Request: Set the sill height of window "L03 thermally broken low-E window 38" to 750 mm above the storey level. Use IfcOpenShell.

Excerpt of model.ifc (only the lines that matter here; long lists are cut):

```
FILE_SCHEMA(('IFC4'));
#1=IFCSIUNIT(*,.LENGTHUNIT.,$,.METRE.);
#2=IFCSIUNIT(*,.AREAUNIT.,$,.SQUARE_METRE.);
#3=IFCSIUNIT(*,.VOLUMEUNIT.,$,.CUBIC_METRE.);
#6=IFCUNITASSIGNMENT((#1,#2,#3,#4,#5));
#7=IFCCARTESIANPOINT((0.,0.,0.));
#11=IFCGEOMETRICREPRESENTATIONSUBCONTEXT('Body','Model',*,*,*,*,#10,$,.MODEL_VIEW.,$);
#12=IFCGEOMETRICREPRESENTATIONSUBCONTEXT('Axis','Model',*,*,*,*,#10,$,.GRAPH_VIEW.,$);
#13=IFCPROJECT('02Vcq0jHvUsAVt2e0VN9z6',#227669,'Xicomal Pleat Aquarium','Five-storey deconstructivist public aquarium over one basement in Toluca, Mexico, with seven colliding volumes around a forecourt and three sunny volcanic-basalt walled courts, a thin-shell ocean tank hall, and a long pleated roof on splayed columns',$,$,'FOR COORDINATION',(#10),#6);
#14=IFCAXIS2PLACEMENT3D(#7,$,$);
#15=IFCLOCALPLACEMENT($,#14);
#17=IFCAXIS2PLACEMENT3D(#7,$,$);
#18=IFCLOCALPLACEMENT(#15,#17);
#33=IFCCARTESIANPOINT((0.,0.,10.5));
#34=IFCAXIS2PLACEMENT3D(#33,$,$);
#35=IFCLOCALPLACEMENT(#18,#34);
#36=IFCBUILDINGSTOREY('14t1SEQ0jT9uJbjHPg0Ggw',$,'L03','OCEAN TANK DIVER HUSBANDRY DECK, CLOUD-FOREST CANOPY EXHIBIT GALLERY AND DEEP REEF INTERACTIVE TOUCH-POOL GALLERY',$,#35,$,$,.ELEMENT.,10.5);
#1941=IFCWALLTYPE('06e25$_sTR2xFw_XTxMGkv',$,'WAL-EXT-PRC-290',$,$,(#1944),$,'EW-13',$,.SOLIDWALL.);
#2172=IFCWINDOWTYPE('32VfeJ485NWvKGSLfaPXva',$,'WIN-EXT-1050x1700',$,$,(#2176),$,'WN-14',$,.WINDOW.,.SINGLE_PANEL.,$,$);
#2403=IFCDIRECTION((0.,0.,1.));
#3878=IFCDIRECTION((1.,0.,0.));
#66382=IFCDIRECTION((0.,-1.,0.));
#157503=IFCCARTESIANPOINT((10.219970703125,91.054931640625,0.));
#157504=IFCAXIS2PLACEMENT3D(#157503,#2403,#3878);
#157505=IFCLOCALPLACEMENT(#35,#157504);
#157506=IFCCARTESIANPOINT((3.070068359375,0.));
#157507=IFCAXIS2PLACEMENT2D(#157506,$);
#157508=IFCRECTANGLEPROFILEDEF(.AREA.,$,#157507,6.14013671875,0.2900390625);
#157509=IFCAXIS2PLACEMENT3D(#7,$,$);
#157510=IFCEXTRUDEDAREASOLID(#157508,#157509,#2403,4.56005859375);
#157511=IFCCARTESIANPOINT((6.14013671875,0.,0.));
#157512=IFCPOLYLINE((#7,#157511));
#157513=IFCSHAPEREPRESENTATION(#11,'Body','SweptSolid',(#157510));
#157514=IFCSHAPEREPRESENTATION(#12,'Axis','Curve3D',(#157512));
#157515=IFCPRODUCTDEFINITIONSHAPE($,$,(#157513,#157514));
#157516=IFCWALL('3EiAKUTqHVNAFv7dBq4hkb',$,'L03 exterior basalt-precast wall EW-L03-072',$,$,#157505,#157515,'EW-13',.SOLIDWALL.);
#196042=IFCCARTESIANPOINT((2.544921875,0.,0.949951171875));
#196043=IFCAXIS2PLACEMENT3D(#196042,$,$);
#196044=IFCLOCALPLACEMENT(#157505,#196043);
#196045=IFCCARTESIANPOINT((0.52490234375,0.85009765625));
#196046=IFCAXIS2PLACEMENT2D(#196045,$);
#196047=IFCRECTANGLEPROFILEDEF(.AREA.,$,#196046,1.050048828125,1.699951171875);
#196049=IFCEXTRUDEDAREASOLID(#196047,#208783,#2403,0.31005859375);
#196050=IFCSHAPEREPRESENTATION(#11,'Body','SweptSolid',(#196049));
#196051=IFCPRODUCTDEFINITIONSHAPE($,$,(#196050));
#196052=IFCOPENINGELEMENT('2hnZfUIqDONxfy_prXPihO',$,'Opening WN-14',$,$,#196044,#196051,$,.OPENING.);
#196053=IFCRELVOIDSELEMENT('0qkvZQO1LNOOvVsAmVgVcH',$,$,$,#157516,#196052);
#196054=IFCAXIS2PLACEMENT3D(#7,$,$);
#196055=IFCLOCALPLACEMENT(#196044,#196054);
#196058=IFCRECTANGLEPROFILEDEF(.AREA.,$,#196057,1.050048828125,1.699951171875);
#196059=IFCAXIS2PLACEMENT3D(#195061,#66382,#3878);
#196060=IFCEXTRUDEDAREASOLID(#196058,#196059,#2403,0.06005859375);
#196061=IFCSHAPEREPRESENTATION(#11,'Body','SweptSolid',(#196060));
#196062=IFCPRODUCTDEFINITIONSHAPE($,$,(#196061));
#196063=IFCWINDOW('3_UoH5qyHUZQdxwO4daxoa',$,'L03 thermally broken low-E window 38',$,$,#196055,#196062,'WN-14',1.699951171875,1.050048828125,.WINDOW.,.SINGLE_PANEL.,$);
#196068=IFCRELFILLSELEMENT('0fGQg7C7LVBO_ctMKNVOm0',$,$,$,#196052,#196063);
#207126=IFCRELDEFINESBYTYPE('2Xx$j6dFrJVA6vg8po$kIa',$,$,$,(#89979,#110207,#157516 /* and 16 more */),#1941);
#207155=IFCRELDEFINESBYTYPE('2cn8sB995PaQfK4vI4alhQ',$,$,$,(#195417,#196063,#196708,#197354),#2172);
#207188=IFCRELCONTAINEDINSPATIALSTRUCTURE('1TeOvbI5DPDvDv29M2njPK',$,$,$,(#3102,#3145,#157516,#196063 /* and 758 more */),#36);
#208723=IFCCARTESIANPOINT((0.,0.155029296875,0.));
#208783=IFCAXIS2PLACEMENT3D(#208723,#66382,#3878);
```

```python
import numpy as np
import ifcopenshell
import ifcopenshell.api.geometry
import ifcopenshell.geom
import ifcopenshell.util.element
import ifcopenshell.util.placement
import ifcopenshell.util.shape
import ifcopenshell.util.unit

model = ifcopenshell.open("model.ifc")
unit_scale = ifcopenshell.util.unit.calculate_unit_scale(model)

window = model.by_guid("3_UoH5qyHUZQdxwO4daxoa")
opening = window.FillsVoids[0].RelatingOpeningElement
storey = ifcopenshell.util.element.get_container(window, ifc_class="IfcBuildingStorey")
level = ifcopenshell.util.placement.get_local_placement(storey.ObjectPlacement)[2, 3]

# The opening's origin need not be at the sill, so measure its lowest point.
shape = ifcopenshell.geom.create_shape(ifcopenshell.geom.settings(), opening)
bottom = ifcopenshell.util.shape.get_shape_bottom_elevation(shape, shape.geometry) / unit_scale
dz = level + 0.75 - bottom

shift = np.array([0.0, 0.0, dz])
# The window is placed relative to its opening, so it follows when the opening moves.
matrix = ifcopenshell.util.placement.get_local_placement(opening.ObjectPlacement)
matrix[:3, 3] += shift
ifcopenshell.api.geometry.edit_object_placement(
    model, product=opening, matrix=matrix, is_si=False, should_transform_children=True
)

print(f"moved by {dz * unit_scale:+.3f} m")

model.write("model_rev.ifc")
```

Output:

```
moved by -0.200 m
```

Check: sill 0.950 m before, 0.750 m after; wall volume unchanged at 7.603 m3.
